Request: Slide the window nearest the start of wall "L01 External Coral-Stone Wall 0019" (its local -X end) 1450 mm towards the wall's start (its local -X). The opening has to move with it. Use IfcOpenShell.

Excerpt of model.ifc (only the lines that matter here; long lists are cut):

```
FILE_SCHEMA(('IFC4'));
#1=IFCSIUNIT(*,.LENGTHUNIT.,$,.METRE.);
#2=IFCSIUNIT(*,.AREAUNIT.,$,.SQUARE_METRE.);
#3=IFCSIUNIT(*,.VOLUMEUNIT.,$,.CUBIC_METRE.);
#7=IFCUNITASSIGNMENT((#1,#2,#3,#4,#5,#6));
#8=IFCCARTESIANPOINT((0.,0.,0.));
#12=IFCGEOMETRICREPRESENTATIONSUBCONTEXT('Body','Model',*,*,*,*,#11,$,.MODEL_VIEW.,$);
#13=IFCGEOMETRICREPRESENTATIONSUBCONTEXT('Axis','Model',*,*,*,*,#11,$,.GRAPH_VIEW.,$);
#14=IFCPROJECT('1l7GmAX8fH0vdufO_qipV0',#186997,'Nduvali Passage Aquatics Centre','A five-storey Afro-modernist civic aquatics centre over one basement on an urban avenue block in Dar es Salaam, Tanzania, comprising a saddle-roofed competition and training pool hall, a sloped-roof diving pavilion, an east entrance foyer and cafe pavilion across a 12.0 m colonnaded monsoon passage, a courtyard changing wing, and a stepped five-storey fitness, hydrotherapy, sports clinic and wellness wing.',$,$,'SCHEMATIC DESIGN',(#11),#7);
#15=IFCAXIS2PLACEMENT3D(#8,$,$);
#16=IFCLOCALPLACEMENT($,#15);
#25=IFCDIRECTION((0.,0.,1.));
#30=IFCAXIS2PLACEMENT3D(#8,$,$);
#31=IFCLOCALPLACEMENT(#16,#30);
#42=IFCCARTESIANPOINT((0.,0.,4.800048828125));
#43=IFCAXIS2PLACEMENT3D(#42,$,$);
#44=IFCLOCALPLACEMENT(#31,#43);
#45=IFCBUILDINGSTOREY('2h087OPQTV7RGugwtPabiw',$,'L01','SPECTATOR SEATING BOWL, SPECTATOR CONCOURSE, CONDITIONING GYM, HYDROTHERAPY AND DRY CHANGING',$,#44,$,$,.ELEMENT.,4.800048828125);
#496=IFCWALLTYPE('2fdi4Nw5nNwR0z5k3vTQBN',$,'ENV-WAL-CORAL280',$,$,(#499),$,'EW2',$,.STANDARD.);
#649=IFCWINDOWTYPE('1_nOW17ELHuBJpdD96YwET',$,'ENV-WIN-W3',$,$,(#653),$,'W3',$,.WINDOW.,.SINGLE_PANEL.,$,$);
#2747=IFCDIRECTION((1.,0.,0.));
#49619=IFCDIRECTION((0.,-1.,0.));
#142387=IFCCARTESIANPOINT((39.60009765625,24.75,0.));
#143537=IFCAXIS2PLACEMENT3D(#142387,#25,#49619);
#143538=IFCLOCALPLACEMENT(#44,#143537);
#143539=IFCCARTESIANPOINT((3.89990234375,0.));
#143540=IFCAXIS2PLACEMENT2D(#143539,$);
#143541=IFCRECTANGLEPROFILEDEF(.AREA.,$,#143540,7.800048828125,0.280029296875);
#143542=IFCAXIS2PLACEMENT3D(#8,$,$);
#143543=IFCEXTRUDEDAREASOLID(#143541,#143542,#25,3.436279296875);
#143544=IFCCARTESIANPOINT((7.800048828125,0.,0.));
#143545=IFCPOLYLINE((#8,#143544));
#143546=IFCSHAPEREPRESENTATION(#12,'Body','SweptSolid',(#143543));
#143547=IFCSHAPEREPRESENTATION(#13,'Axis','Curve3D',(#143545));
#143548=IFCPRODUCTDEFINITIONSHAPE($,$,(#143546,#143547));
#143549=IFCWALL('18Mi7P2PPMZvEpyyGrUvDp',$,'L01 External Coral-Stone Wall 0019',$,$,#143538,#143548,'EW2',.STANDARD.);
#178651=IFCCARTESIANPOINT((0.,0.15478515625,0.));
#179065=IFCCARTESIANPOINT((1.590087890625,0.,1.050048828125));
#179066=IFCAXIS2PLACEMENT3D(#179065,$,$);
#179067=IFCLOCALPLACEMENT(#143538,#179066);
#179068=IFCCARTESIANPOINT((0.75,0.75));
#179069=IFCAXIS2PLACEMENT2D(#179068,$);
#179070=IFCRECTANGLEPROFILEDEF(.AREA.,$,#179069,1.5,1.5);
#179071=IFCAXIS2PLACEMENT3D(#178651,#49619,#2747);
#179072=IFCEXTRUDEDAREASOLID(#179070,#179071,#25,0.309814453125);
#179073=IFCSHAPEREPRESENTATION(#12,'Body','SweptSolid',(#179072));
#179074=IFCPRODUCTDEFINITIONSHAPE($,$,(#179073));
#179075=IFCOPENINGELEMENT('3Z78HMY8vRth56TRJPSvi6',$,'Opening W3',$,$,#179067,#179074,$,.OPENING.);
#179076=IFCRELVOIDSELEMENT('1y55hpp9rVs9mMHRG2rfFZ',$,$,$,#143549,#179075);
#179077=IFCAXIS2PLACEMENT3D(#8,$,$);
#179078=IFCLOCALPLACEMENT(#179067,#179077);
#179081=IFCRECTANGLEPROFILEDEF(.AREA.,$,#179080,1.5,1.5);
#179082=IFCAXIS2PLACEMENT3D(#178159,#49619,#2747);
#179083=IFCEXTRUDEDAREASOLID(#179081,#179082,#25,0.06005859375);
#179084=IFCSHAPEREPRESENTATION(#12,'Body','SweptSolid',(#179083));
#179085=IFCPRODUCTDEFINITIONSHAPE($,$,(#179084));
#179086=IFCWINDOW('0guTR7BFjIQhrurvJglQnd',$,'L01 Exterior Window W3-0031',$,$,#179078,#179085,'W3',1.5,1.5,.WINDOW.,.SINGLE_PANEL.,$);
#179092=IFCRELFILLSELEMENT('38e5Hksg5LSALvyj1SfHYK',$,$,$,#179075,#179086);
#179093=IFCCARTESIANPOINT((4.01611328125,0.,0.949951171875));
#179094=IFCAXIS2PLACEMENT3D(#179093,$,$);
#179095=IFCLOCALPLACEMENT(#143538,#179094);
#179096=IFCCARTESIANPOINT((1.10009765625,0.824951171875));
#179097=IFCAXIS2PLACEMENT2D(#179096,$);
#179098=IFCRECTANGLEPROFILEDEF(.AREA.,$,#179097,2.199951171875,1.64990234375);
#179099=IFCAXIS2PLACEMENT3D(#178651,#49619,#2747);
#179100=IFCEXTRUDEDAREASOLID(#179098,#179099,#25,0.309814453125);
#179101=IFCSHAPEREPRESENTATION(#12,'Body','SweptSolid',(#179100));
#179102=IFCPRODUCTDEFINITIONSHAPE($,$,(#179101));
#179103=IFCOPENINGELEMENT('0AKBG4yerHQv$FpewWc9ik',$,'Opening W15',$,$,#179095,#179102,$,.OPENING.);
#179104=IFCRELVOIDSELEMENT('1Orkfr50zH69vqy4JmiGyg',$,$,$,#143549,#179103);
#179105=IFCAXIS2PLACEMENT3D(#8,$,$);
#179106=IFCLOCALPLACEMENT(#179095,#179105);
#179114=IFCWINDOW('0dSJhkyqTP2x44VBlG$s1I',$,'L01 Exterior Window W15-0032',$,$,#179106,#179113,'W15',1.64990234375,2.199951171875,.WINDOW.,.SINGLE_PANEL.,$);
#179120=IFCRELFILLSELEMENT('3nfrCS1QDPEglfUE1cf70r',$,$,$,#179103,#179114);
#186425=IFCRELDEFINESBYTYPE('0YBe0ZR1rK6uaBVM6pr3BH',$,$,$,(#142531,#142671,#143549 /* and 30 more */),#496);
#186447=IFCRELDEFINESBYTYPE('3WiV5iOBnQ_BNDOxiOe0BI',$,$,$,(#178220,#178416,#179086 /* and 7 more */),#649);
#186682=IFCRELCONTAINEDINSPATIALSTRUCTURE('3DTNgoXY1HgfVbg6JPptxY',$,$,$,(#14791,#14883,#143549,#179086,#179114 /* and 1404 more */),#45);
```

```python
import ifcopenshell
import ifcopenshell.api.geometry
import ifcopenshell.util.placement
import ifcopenshell.util.unit

model = ifcopenshell.open("model.ifc")
unit_scale = ifcopenshell.util.unit.calculate_unit_scale(model)

window = model.by_guid("0guTR7BFjIQhrurvJglQnd")
opening = window.FillsVoids[0].RelatingOpeningElement
wall = opening.VoidsElements[0].RelatingBuildingElement

wall_matrix = ifcopenshell.util.placement.get_local_placement(wall.ObjectPlacement)
shift = wall_matrix[:3, 0] * -1.45 / unit_scale
before = ifcopenshell.util.placement.get_local_placement(window.ObjectPlacement)[:3, 3].copy()

# The window is placed relative to its opening, so it follows when the opening moves.
matrix = ifcopenshell.util.placement.get_local_placement(opening.ObjectPlacement)
matrix[:3, 3] += shift
ifcopenshell.api.geometry.edit_object_placement(
    model, product=opening, matrix=matrix, is_si=False, should_transform_children=True
)

after = ifcopenshell.util.placement.get_local_placement(window.ObjectPlacement)[:3, 3]
print("window moved by", (after - before).round(3) + 0.0)

model.write("model-out.ifc")
```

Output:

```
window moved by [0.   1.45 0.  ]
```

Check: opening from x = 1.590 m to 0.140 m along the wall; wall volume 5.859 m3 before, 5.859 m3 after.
